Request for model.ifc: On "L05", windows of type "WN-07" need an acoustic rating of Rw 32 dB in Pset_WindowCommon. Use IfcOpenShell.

First a look at what the model holds.

```python
import ifcopenshell
import ifcopenshell.util.element

model = ifcopenshell.open("model.ifc")
print(model.schema)
storey = next(s for s in model.by_type("IfcBuildingStorey") if s.Name == "L05")
windows = [e for e in ifcopenshell.util.element.get_decomposition(storey) if e.is_a("IfcWindow")]
seen = {}
for e in windows:
    element_type = ifcopenshell.util.element.get_type(e)
    key = (element_type.Name if element_type != e and element_type else None, ifcopenshell.util.element.get_pset(e, "Pset_WindowCommon", "AcousticRating"))
    seen[key] = seen.get(key, 0) + 1
for (name, value), count in sorted(seen.items(), key=str):
    print(count, "x", name, "|", value)
```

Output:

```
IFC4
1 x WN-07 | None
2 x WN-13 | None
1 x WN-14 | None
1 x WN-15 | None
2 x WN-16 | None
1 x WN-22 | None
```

```python
import ifcopenshell
import ifcopenshell.api.pset
import ifcopenshell.util.element

model = ifcopenshell.open("model.ifc")

storey = next(s for s in model.by_type("IfcBuildingStorey") if s.Name == "L05")
windows = [e for e in ifcopenshell.util.element.get_decomposition(storey) if e.is_a("IfcWindow")]

count = 0
for e in windows:
    element_type = ifcopenshell.util.element.get_type(e)
    if element_type in (None, e) or element_type.Name != "WN-07":
        continue
    # add_pset returns the element's existing set when there is one.
    pset = ifcopenshell.api.pset.add_pset(model, product=e, name="Pset_WindowCommon")
    ifcopenshell.api.pset.edit_pset(model, pset=pset, properties={"AcousticRating": "Rw 32 dB"})
    count += 1

print(count, "windows updated")

model.write("model_edited.ifc")
```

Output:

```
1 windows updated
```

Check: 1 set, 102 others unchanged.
